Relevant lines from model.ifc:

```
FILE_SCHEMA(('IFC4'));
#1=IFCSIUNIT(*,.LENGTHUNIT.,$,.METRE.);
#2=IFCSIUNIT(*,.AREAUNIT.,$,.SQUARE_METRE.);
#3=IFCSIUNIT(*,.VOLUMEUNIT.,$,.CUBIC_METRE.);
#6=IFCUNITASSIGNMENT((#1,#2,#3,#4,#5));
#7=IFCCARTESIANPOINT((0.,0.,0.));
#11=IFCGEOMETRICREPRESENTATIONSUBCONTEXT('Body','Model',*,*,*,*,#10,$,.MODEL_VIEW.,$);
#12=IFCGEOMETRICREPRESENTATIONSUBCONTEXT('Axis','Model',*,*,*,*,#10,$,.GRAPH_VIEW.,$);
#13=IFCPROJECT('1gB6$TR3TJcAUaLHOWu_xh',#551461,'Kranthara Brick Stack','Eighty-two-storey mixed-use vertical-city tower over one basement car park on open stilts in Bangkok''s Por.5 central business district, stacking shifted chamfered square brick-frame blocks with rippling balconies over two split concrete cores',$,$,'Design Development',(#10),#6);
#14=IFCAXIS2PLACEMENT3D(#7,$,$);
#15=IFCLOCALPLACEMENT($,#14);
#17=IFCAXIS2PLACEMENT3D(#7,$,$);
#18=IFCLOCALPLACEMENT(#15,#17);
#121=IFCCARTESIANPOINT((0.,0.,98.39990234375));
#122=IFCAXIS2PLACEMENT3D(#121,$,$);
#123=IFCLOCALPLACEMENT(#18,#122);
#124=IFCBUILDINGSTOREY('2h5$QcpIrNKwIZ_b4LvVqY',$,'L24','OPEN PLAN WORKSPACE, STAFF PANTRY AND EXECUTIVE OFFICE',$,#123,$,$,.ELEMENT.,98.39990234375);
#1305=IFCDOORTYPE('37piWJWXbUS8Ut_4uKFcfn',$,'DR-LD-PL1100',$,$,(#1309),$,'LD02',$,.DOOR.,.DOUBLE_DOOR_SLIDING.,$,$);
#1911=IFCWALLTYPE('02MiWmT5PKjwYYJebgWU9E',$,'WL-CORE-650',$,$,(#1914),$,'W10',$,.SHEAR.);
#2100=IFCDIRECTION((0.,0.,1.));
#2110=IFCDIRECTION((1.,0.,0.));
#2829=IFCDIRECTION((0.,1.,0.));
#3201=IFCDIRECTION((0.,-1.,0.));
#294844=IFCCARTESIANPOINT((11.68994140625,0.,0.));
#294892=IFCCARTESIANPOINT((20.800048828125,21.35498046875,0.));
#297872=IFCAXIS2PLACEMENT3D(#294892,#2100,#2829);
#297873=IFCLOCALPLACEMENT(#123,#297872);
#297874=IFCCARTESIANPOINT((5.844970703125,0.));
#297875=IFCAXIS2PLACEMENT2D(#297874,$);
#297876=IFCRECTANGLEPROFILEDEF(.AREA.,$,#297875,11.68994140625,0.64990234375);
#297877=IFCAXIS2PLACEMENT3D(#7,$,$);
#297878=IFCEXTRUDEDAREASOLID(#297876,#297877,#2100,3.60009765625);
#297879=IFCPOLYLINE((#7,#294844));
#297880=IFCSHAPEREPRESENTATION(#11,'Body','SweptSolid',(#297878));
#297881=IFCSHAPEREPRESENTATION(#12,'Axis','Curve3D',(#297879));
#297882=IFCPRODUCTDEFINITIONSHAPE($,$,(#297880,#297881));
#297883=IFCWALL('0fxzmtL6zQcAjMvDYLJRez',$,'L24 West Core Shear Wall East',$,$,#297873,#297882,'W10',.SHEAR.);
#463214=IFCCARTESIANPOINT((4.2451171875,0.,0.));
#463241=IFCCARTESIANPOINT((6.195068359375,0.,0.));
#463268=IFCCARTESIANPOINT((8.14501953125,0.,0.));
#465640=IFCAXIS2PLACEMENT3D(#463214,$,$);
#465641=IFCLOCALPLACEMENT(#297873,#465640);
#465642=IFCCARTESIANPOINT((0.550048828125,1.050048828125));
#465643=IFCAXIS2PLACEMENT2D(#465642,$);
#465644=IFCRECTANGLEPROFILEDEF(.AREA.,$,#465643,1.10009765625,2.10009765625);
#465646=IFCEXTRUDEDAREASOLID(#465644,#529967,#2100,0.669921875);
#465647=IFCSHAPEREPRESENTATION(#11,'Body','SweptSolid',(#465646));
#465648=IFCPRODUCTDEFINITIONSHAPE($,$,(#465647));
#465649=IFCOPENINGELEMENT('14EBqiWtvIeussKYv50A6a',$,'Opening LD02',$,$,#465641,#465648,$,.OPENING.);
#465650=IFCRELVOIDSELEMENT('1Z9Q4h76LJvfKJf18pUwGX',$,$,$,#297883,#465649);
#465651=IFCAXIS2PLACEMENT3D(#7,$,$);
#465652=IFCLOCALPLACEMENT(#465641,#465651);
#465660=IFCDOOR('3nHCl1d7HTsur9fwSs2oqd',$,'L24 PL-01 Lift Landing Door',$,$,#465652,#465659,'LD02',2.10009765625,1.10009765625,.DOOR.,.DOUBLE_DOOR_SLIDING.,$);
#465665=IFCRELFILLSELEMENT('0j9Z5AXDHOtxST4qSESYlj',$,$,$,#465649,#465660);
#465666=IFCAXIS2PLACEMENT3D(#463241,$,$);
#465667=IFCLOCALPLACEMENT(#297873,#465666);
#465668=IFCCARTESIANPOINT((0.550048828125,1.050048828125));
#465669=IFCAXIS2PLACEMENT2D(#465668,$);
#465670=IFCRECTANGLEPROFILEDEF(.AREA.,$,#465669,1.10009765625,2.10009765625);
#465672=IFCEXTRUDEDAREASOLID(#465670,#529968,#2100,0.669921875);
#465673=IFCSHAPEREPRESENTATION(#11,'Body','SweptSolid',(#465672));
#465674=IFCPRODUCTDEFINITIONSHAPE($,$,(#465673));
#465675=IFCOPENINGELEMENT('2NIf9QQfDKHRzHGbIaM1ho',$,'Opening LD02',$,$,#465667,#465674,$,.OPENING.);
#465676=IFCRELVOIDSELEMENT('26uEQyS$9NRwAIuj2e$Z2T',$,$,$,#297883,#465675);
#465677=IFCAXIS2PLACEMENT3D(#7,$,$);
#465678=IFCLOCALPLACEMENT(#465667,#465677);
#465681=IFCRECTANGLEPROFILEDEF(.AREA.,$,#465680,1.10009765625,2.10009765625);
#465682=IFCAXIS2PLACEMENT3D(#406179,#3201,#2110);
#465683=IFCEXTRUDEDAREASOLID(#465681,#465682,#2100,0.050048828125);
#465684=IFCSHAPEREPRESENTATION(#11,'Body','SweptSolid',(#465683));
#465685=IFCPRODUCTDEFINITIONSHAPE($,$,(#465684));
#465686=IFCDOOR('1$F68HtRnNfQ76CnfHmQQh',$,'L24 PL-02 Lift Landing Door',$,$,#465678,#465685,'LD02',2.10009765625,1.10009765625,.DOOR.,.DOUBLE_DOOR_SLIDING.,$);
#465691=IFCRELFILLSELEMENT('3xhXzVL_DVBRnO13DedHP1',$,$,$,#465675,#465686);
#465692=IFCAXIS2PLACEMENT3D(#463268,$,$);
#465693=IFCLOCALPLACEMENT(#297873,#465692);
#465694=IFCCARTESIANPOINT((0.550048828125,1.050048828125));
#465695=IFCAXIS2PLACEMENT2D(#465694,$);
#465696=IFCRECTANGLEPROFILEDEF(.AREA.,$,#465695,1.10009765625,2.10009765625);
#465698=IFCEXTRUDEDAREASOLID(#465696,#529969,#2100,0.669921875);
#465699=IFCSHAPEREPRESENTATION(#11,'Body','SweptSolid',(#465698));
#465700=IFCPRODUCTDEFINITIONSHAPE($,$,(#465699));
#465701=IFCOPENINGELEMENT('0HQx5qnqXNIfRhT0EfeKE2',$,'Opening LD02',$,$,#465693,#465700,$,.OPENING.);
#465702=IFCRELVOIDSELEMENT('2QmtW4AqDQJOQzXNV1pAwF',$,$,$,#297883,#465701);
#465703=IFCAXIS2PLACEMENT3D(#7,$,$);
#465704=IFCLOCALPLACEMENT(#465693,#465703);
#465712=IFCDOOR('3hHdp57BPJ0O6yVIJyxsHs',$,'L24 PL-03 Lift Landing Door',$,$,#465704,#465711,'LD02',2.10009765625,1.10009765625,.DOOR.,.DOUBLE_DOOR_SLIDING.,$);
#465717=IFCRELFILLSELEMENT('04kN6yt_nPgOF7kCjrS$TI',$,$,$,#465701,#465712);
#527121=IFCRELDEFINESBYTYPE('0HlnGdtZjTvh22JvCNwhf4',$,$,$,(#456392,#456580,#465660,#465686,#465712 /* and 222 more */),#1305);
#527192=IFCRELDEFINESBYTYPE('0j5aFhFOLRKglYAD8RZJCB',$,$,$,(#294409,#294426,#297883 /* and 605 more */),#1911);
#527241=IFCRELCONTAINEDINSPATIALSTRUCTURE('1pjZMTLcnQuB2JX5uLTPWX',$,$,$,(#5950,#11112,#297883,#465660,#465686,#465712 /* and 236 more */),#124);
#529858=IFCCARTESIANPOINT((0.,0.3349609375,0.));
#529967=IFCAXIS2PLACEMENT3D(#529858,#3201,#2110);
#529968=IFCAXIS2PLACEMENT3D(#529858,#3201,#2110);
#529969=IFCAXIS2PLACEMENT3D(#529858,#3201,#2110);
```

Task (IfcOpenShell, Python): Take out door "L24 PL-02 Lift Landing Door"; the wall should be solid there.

```python
import ifcopenshell
import ifcopenshell.api.feature
import ifcopenshell.api.root
import ifcopenshell.geom
import ifcopenshell.util.shape

model = ifcopenshell.open("model.ifc")
settings = ifcopenshell.geom.settings()


def volume(element):
    """Net volume in cubic metres, openings subtracted."""
    shape = ifcopenshell.geom.create_shape(settings, element)
    return ifcopenshell.util.shape.get_volume(shape.geometry)


door = model.by_id(465686)
opening = door.FillsVoids[0].RelatingOpeningElement
wall = opening.VoidsElements[0].RelatingBuildingElement
before = volume(wall)

ifcopenshell.api.root.remove_product(model, product=door)
ifcopenshell.api.feature.remove_feature(model, feature=opening)

after = volume(wall)

print(f"wall volume {before:.3f} -> {after:.3f} m3")

model.write("model_edited.ifc")
```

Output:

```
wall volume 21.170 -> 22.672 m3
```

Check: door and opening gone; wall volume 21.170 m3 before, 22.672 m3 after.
